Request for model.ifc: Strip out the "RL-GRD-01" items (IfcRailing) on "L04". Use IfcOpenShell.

First a look at what the model holds.

```python
import ifcopenshell
import ifcopenshell.util.element

model = ifcopenshell.open("model.ifc")
print(model.schema)
storey = next(s for s in model.by_type("IfcBuildingStorey") if s.Name == "L04")
railings = [e for e in ifcopenshell.util.element.get_decomposition(storey) if e.is_a("IfcRailing")]
seen = {}
for e in railings:
    element_type = ifcopenshell.util.element.get_type(e)
    name = element_type.Name if element_type not in (None, e) else None
    seen[name] = seen.get(name, 0) + 1
for name, count in sorted(seen.items(), key=str):
    print(count, "x", name)
```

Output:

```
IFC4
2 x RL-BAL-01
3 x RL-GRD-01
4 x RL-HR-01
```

```python
import ifcopenshell
import ifcopenshell.api.root
import ifcopenshell.util.element

model = ifcopenshell.open("model.ifc")

storey = next(s for s in model.by_type("IfcBuildingStorey") if s.Name == "L04")
railings = [e for e in ifcopenshell.util.element.get_decomposition(storey) if e.is_a("IfcRailing")]
targets = [e for e in railings if (t := ifcopenshell.util.element.get_type(e)) not in (None, e) and t.Name == "RL-GRD-01"]

for e in targets:
    ifcopenshell.api.root.remove_product(model, product=e)
print(len(targets), "removed")

model.write("model_updated.ifc")
```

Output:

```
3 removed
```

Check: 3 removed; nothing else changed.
